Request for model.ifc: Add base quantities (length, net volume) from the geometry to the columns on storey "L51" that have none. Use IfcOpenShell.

First a look at what the model holds.

```python
import ifcopenshell
import ifcopenshell.util.element
import ifcopenshell.util.unit

model = ifcopenshell.open("model.ifc")
print(model.schema)
for unit_type in ("LENGTHUNIT", "AREAUNIT", "VOLUMEUNIT"):
    print(unit_type, ifcopenshell.util.unit.calculate_unit_scale(model, unit_type))
storey = next(s for s in model.by_type("IfcBuildingStorey") if s.Name == "L51")
columns = [e for e in ifcopenshell.util.element.get_decomposition(storey) if e.is_a("IfcColumn")]
for e in sorted(columns, key=lambda e: e.id()):
    print(e.id(), e.is_a(), e.Name, list(ifcopenshell.util.element.get_psets(e, qtos_only=True)), sep=" | ")
```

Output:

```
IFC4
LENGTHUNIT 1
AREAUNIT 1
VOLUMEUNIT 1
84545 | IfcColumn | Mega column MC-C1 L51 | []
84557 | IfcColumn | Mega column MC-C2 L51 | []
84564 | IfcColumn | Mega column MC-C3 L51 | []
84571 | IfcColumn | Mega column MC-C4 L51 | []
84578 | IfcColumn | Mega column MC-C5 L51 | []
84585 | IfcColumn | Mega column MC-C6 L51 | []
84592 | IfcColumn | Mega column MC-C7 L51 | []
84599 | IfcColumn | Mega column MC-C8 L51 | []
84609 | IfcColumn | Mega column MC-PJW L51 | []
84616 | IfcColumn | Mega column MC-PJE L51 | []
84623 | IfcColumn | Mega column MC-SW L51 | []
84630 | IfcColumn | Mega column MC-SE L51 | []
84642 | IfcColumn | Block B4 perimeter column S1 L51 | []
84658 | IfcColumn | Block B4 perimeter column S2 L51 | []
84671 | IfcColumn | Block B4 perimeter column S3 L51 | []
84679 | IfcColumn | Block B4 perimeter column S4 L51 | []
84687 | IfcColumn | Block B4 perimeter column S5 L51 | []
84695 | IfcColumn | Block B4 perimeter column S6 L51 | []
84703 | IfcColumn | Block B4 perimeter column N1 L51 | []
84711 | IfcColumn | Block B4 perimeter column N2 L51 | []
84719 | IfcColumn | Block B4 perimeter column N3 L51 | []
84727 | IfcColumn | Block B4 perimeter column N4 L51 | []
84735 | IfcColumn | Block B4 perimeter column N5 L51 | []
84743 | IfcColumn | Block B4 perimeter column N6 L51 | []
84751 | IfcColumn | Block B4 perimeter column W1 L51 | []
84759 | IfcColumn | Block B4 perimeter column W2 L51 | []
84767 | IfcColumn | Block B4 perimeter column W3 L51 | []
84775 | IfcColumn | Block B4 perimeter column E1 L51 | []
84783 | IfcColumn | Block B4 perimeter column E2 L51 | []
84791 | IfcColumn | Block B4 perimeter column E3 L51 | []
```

```python
import ifcopenshell
import ifcopenshell.api.pset
import ifcopenshell.geom
import ifcopenshell.util.element
import ifcopenshell.util.shape
import ifcopenshell.util.unit

model = ifcopenshell.open("model.ifc")
unit_scale = ifcopenshell.util.unit.calculate_unit_scale(model)
volume_scale = ifcopenshell.util.unit.calculate_unit_scale(model, "VOLUMEUNIT")
settings = ifcopenshell.geom.settings()

storey = next(s for s in model.by_type("IfcBuildingStorey") if s.Name == "L51")
columns = [e for e in ifcopenshell.util.element.get_decomposition(storey) if e.is_a("IfcColumn")]

for e in sorted(columns, key=lambda e: e.id()):
    if ifcopenshell.util.element.get_psets(e, qtos_only=True, should_inherit=False):
        continue
    # Geometry comes back in metres, in the element's own axes.
    shape = ifcopenshell.geom.create_shape(settings, e)
    values = {
        "Length": ifcopenshell.util.shape.get_z(shape.geometry) / unit_scale,
        "NetVolume": ifcopenshell.util.shape.get_volume(shape.geometry) / volume_scale,
    }
    qto = ifcopenshell.api.pset.add_qto(model, product=e, name="Qto_ColumnBaseQuantities")
    ifcopenshell.api.pset.edit_qto(model, qto=qto, properties=values)
    print(e.id(), {k: round(v, 3) for k, v in values.items()})

model.write("model_edited.ifc")
```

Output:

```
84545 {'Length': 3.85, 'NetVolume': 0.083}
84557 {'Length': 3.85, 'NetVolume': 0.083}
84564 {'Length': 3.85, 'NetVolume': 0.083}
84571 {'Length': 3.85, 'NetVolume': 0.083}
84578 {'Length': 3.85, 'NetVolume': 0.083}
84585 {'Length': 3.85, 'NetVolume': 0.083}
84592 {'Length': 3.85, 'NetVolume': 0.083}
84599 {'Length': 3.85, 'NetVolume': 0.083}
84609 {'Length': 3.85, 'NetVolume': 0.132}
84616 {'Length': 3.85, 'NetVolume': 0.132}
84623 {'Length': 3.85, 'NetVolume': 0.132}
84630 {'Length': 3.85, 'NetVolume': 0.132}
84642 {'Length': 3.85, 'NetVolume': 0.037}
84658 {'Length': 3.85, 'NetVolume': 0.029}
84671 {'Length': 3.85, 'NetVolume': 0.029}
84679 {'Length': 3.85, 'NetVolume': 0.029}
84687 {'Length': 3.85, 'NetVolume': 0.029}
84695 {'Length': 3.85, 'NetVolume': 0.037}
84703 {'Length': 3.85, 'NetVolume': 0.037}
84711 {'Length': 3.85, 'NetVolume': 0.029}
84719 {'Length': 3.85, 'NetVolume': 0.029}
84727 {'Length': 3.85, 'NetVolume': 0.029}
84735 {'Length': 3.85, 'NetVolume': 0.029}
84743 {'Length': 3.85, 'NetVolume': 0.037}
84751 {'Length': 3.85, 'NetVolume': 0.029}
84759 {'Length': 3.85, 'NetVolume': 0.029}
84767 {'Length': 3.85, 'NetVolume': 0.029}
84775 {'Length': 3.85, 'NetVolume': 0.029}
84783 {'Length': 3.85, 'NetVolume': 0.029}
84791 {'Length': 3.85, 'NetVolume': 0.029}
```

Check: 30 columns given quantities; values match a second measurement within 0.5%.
